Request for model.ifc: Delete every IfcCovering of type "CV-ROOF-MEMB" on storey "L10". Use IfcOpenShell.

First a look at what the model holds.

```python
import ifcopenshell
import ifcopenshell.util.element

model = ifcopenshell.open("model.ifc")
print(model.schema)
storey = next(s for s in model.by_type("IfcBuildingStorey") if s.Name == "L10")
coverings = [e for e in ifcopenshell.util.element.get_decomposition(storey) if e.is_a("IfcCovering")]
seen = {}
for e in coverings:
    element_type = ifcopenshell.util.element.get_type(e)
    name = element_type.Name if element_type not in (None, e) else None
    seen[name] = seen.get(name, 0) + 1
for name, count in sorted(seen.items(), key=str):
    print(count, "x", name)
```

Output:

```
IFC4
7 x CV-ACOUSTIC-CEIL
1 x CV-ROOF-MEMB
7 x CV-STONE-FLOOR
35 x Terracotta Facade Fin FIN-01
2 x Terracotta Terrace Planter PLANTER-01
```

```python
import ifcopenshell
import ifcopenshell.api.root
import ifcopenshell.util.element

model = ifcopenshell.open("model.ifc")

storey = next(s for s in model.by_type("IfcBuildingStorey") if s.Name == "L10")
coverings = [e for e in ifcopenshell.util.element.get_decomposition(storey) if e.is_a("IfcCovering")]
targets = [e for e in coverings if (t := ifcopenshell.util.element.get_type(e)) not in (None, e) and t.Name == "CV-ROOF-MEMB"]

for e in targets:
    ifcopenshell.api.root.remove_product(model, product=e)
print(len(targets), "removed")

model.write("model_rev.ifc")
```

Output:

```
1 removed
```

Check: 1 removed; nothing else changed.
